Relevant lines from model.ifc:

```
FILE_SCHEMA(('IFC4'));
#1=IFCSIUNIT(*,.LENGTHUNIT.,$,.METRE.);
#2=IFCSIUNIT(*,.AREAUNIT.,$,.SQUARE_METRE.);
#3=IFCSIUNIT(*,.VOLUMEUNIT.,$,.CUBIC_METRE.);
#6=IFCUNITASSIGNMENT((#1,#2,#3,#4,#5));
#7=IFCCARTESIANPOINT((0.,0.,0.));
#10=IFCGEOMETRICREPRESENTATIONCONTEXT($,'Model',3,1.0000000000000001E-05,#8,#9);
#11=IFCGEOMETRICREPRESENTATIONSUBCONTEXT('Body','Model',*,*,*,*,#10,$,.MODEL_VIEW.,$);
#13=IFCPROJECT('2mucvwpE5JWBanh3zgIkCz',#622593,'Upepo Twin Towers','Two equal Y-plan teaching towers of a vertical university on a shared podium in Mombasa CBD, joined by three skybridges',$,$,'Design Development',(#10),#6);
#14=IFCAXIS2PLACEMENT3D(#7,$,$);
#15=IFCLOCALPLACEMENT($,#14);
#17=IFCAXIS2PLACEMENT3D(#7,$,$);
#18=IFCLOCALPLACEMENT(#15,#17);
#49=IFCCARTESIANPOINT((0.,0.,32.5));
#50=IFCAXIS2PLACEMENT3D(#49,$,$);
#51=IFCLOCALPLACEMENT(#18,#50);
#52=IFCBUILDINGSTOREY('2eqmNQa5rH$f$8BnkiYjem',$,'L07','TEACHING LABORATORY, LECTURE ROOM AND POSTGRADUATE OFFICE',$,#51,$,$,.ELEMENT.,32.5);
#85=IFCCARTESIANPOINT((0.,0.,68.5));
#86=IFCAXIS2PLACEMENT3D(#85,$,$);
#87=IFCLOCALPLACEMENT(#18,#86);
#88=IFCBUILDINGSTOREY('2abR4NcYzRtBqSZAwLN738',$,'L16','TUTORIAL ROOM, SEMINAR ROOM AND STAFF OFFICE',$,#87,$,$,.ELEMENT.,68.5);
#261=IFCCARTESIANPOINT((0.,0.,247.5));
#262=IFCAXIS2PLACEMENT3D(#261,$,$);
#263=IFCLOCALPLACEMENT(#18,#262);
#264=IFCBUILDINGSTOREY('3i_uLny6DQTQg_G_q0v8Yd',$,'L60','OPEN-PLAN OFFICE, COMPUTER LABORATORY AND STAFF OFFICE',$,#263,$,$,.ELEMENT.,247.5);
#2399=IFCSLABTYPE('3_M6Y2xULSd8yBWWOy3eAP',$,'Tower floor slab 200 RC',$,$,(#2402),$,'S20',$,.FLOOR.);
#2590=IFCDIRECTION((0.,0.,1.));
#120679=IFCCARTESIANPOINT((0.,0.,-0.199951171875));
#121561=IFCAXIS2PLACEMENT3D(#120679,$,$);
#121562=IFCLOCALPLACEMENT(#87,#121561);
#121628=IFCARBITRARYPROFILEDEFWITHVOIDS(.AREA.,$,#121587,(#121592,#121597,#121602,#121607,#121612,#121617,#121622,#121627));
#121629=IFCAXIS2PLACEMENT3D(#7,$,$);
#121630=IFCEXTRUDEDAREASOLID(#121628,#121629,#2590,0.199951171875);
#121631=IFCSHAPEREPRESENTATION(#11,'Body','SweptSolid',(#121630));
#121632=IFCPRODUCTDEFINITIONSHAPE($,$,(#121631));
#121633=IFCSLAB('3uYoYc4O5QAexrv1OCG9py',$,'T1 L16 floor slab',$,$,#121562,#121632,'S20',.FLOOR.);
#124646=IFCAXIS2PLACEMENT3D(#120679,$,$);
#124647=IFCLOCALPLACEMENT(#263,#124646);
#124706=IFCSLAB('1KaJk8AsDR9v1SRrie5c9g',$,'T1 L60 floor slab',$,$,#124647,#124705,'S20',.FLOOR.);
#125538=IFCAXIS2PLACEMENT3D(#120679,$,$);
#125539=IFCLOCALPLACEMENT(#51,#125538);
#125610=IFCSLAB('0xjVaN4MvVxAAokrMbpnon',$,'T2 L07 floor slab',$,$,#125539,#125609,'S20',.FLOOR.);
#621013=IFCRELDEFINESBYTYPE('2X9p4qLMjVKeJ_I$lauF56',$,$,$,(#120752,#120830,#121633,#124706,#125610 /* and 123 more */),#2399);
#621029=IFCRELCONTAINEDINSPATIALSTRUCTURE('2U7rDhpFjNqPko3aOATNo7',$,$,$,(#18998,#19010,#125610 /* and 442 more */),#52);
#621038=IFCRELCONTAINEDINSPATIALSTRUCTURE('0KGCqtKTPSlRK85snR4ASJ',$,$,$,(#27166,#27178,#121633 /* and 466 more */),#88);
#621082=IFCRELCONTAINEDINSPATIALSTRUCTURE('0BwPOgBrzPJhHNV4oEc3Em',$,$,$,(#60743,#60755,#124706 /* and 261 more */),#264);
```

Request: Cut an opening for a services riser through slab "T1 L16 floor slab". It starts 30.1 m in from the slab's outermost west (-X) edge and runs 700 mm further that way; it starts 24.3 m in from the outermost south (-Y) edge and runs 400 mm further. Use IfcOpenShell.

```python
import numpy as np
import ifcopenshell
import ifcopenshell.api.feature
import ifcopenshell.api.geometry
import ifcopenshell.api.root
import ifcopenshell.geom
import ifcopenshell.util.placement
import ifcopenshell.util.representation
import ifcopenshell.util.shape
import ifcopenshell.util.unit

model = ifcopenshell.open("model.ifc")
unit_scale = ifcopenshell.util.unit.calculate_unit_scale(model)
settings = ifcopenshell.geom.settings()


def volume(element):
    """Net volume in cubic metres, openings subtracted."""
    shape = ifcopenshell.geom.create_shape(settings, element)
    return ifcopenshell.util.shape.get_volume(shape.geometry)


slab = model.by_guid("3uYoYc4O5QAexrv1OCG9py")
before = volume(slab)

# Extent in the slab's own axes, in metres. The edges named are its -X and -Y sides.
slab_shape = ifcopenshell.geom.create_shape(settings, slab)
vertices = ifcopenshell.util.shape.get_vertices(slab_shape.geometry)
x_min, y_min, bottom = vertices.min(axis=0)
top = vertices[:, 2].max()

opening = ifcopenshell.api.root.create_entity(model, ifc_class="IfcOpeningElement", name="Services riser opening", predefined_type="OPENING")
context = ifcopenshell.util.representation.get_context(model, "Model", "Body", "MODEL_VIEW")
width, depth = 0.7, 0.4
outline = [(0.0, 0.0), (width, 0.0), (width, depth), (0.0, depth), (0.0, 0.0)]
# Overshoot both faces by 50 mm so the cut is clean.
shape = ifcopenshell.api.geometry.add_slab_representation(
    model, context=context, depth=top - bottom + 0.1, polyline=outline
)
ifcopenshell.api.geometry.assign_representation(model, product=opening, representation=shape)

matrix = ifcopenshell.util.placement.get_local_placement(slab.ObjectPlacement)
matrix[:, 3] = matrix @ np.append(np.array([x_min + 30.1, y_min + 24.3, bottom - 0.05]) / unit_scale, 1.0)
ifcopenshell.api.geometry.edit_object_placement(model, product=opening, matrix=matrix, is_si=False)
ifcopenshell.api.feature.add_feature(model, feature=opening, element=slab)

after = volume(slab)

print(f"slab volume {before:.3f} -> {after:.3f} m3")

model.write("model_updated.ifc")
```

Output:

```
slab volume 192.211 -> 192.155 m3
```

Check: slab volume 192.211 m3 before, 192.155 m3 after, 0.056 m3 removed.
